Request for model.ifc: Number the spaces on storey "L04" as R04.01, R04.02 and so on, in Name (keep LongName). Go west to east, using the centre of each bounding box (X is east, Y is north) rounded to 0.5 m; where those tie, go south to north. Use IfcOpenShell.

First a look at what the model holds.

```python
import ifcopenshell
import ifcopenshell.util.element
import ifcopenshell.util.placement

model = ifcopenshell.open("model.ifc")
print(model.schema)
storey = next(s for s in model.by_type("IfcBuildingStorey") if s.Name == "L04")
spaces = [e for e in ifcopenshell.util.element.get_decomposition(storey) if e.is_a("IfcSpace")]
for e in sorted(spaces, key=lambda e: e.id()):
    origin = ifcopenshell.util.placement.get_local_placement(e.ObjectPlacement)[:3, 3]
    print(e.id(), e.Name, e.LongName, origin.round(2) + 0.0, sep=" | ")
```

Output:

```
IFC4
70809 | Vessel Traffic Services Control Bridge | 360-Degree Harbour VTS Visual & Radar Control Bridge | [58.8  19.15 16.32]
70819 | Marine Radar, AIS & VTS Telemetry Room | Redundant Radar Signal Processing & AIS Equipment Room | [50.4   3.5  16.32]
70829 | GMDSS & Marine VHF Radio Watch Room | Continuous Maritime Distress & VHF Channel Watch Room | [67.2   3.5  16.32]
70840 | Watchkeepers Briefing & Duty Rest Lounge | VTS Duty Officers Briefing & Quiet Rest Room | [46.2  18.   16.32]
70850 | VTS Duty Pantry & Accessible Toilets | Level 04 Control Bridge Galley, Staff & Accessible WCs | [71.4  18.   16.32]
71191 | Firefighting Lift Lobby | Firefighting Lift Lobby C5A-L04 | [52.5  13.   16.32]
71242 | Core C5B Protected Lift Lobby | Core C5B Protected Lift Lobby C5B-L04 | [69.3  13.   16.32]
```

```python
import ifcopenshell
import ifcopenshell.geom
import ifcopenshell.util.element
import ifcopenshell.util.shape

model = ifcopenshell.open("model.ifc")
settings = ifcopenshell.geom.settings()
settings.set("use-world-coords", True)


def centre(element):
    shape = ifcopenshell.geom.create_shape(settings, element)
    return ifcopenshell.util.shape.get_bbox_centroid(shape.geometry)


storey = next(s for s in model.by_type("IfcBuildingStorey") if s.Name == "L04")
spaces = [e for e in ifcopenshell.util.element.get_decomposition(storey) if e.is_a("IfcSpace")]

# Insertion points can sit at a corner or the storey origin, so sort by the geometry (in metres).
centres = {e: centre(e) for e in spaces}
spaces.sort(key=lambda e: (round(centres[e][0] / 0.5), centres[e][1]))

for i, e in enumerate(spaces, start=1):
    number = f"R04.{i:02d}"
    e.Name = number
    print(e.id(), number)

model.write("model-out.ifc")
```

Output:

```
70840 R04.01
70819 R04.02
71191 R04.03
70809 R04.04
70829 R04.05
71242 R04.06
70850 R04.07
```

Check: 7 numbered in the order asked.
